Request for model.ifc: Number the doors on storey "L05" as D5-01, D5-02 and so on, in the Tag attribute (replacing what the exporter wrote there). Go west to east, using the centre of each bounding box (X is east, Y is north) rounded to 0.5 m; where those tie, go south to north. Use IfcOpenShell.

First a look at what the model holds.

```python
import ifcopenshell
import ifcopenshell.util.element
import ifcopenshell.util.placement

model = ifcopenshell.open("model.ifc")
print(model.schema)
storey = next(s for s in model.by_type("IfcBuildingStorey") if s.Name == "L05")
doors = [e for e in ifcopenshell.util.element.get_decomposition(storey) if e.is_a("IfcDoor")]
for e in sorted(doors, key=lambda e: e.id()):
    origin = ifcopenshell.util.placement.get_local_placement(e.ObjectPlacement)[:3, 3]
    print(e.id(), e.Tag, e.Name, origin.round(2) + 0.0, sep=" | ")
```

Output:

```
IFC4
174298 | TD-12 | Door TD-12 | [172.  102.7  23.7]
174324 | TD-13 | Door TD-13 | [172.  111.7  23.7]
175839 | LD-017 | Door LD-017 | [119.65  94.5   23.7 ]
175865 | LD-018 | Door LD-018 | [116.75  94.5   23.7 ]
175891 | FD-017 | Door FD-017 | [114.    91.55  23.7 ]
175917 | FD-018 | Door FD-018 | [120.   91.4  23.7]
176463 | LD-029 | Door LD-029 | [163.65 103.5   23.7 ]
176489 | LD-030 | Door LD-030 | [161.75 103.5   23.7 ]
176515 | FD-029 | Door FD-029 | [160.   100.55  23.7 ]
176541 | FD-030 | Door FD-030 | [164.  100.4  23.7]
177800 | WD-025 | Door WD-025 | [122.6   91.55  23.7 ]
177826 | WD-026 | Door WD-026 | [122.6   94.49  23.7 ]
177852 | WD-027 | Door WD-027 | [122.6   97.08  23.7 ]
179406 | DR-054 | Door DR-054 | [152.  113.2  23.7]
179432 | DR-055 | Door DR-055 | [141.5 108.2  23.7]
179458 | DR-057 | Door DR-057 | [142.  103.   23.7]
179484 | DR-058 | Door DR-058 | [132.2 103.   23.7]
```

```python
import ifcopenshell
import ifcopenshell.geom
import ifcopenshell.util.element
import ifcopenshell.util.shape

model = ifcopenshell.open("model.ifc")
settings = ifcopenshell.geom.settings()
settings.set("use-world-coords", True)


def centre(element):
    shape = ifcopenshell.geom.create_shape(settings, element)
    return ifcopenshell.util.shape.get_bbox_centroid(shape.geometry)


storey = next(s for s in model.by_type("IfcBuildingStorey") if s.Name == "L05")
doors = [e for e in ifcopenshell.util.element.get_decomposition(storey) if e.is_a("IfcDoor")]

# Insertion points can sit at a corner or the storey origin, so sort by the geometry (in metres).
centres = {e: centre(e) for e in doors}
doors.sort(key=lambda e: (round(centres[e][0] / 0.5), centres[e][1]))

for i, e in enumerate(doors, start=1):
    number = f"D5-{i:02d}"
    e.Tag = number
    print(e.id(), number)

model.write("model_rev.ifc")
```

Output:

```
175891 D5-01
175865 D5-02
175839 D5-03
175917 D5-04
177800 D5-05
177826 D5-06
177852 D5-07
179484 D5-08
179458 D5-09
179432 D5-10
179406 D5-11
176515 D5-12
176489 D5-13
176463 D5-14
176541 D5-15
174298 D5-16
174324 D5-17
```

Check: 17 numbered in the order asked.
